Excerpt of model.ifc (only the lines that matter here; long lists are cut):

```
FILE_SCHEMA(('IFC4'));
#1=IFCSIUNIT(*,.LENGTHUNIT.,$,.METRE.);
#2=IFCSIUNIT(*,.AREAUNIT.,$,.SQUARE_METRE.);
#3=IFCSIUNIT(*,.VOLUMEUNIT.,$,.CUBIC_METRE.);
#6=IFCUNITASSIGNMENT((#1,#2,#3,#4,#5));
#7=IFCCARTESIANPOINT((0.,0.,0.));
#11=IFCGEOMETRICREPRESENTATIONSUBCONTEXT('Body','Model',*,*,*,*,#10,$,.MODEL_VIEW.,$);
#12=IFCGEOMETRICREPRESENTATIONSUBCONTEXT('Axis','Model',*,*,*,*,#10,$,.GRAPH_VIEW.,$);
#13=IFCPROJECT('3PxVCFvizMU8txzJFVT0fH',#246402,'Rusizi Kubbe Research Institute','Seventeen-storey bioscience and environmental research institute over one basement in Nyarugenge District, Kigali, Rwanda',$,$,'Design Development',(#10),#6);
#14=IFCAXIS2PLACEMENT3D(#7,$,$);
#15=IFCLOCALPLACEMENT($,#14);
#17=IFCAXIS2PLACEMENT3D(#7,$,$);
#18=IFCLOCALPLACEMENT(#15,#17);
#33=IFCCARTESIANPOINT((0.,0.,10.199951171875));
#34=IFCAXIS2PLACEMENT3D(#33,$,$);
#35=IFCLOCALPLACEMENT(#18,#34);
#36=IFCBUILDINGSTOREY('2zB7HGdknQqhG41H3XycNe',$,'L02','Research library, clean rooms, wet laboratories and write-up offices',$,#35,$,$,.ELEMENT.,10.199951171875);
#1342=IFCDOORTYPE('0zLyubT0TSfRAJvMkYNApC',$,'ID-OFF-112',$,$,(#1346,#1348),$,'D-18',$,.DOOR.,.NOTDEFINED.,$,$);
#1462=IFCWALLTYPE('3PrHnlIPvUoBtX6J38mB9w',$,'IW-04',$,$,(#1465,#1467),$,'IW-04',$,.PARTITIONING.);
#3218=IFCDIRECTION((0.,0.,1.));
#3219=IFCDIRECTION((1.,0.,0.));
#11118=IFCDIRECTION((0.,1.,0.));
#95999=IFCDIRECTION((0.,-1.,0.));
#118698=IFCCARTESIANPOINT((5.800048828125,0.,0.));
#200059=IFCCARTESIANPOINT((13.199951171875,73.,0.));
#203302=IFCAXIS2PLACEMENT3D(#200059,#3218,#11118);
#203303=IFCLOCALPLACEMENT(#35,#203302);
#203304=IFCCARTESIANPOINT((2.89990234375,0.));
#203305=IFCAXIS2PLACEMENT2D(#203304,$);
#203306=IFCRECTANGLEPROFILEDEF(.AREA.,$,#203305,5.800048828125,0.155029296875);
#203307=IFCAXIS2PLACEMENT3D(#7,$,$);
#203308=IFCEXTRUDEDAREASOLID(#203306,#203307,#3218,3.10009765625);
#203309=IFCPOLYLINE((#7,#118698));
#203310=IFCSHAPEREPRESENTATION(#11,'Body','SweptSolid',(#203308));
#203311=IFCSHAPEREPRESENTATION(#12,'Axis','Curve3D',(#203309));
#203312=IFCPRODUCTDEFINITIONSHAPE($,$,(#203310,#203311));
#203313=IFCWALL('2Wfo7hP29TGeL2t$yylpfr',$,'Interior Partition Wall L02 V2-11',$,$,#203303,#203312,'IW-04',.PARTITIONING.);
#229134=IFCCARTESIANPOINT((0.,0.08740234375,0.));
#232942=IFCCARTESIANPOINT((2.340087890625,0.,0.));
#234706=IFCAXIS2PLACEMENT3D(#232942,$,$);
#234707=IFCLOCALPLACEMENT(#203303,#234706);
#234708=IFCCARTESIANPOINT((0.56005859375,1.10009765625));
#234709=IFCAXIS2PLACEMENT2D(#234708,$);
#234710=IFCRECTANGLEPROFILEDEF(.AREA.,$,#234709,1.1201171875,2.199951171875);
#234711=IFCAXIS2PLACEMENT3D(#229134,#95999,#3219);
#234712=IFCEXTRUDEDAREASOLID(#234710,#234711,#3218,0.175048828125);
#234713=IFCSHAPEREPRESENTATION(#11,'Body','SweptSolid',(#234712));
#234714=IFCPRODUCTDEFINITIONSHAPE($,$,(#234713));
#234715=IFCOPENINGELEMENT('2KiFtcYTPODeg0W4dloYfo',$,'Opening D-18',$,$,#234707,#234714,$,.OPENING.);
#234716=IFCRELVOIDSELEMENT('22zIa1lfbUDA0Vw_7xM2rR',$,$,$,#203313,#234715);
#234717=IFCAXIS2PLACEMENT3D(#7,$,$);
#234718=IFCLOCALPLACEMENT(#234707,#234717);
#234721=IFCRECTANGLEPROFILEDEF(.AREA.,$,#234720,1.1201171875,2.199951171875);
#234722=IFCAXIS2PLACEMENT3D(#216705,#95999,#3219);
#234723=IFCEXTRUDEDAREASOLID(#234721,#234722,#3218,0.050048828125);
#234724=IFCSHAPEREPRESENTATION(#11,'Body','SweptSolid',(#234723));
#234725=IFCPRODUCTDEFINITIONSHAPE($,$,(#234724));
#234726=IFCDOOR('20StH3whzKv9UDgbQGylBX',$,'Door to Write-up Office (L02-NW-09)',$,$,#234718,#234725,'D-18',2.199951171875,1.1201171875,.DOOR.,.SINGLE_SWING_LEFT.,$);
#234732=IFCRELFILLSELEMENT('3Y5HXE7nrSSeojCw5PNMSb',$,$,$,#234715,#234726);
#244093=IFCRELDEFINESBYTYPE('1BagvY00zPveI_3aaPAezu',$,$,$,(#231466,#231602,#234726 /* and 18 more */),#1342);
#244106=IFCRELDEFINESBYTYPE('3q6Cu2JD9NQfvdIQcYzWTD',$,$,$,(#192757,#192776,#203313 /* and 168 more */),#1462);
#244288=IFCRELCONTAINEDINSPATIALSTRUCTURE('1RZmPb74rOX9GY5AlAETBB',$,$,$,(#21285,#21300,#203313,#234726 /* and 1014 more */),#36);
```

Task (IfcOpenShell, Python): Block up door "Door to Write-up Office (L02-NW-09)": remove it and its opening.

```python
import ifcopenshell
import ifcopenshell.api.feature
import ifcopenshell.api.root
import ifcopenshell.geom
import ifcopenshell.util.shape

model = ifcopenshell.open("model.ifc")
settings = ifcopenshell.geom.settings()


def volume(element):
    """Net volume in cubic metres, openings subtracted."""
    shape = ifcopenshell.geom.create_shape(settings, element)
    return ifcopenshell.util.shape.get_volume(shape.geometry)


door = model.by_id(234726)
opening = door.FillsVoids[0].RelatingOpeningElement
wall = opening.VoidsElements[0].RelatingBuildingElement
before = volume(wall)

ifcopenshell.api.root.remove_product(model, product=door)
ifcopenshell.api.feature.remove_feature(model, feature=opening)

after = volume(wall)

print(f"wall volume {before:.3f} -> {after:.3f} m3")

model.write("model_edited.ifc")
```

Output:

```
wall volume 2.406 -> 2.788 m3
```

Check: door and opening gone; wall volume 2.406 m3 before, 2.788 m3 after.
